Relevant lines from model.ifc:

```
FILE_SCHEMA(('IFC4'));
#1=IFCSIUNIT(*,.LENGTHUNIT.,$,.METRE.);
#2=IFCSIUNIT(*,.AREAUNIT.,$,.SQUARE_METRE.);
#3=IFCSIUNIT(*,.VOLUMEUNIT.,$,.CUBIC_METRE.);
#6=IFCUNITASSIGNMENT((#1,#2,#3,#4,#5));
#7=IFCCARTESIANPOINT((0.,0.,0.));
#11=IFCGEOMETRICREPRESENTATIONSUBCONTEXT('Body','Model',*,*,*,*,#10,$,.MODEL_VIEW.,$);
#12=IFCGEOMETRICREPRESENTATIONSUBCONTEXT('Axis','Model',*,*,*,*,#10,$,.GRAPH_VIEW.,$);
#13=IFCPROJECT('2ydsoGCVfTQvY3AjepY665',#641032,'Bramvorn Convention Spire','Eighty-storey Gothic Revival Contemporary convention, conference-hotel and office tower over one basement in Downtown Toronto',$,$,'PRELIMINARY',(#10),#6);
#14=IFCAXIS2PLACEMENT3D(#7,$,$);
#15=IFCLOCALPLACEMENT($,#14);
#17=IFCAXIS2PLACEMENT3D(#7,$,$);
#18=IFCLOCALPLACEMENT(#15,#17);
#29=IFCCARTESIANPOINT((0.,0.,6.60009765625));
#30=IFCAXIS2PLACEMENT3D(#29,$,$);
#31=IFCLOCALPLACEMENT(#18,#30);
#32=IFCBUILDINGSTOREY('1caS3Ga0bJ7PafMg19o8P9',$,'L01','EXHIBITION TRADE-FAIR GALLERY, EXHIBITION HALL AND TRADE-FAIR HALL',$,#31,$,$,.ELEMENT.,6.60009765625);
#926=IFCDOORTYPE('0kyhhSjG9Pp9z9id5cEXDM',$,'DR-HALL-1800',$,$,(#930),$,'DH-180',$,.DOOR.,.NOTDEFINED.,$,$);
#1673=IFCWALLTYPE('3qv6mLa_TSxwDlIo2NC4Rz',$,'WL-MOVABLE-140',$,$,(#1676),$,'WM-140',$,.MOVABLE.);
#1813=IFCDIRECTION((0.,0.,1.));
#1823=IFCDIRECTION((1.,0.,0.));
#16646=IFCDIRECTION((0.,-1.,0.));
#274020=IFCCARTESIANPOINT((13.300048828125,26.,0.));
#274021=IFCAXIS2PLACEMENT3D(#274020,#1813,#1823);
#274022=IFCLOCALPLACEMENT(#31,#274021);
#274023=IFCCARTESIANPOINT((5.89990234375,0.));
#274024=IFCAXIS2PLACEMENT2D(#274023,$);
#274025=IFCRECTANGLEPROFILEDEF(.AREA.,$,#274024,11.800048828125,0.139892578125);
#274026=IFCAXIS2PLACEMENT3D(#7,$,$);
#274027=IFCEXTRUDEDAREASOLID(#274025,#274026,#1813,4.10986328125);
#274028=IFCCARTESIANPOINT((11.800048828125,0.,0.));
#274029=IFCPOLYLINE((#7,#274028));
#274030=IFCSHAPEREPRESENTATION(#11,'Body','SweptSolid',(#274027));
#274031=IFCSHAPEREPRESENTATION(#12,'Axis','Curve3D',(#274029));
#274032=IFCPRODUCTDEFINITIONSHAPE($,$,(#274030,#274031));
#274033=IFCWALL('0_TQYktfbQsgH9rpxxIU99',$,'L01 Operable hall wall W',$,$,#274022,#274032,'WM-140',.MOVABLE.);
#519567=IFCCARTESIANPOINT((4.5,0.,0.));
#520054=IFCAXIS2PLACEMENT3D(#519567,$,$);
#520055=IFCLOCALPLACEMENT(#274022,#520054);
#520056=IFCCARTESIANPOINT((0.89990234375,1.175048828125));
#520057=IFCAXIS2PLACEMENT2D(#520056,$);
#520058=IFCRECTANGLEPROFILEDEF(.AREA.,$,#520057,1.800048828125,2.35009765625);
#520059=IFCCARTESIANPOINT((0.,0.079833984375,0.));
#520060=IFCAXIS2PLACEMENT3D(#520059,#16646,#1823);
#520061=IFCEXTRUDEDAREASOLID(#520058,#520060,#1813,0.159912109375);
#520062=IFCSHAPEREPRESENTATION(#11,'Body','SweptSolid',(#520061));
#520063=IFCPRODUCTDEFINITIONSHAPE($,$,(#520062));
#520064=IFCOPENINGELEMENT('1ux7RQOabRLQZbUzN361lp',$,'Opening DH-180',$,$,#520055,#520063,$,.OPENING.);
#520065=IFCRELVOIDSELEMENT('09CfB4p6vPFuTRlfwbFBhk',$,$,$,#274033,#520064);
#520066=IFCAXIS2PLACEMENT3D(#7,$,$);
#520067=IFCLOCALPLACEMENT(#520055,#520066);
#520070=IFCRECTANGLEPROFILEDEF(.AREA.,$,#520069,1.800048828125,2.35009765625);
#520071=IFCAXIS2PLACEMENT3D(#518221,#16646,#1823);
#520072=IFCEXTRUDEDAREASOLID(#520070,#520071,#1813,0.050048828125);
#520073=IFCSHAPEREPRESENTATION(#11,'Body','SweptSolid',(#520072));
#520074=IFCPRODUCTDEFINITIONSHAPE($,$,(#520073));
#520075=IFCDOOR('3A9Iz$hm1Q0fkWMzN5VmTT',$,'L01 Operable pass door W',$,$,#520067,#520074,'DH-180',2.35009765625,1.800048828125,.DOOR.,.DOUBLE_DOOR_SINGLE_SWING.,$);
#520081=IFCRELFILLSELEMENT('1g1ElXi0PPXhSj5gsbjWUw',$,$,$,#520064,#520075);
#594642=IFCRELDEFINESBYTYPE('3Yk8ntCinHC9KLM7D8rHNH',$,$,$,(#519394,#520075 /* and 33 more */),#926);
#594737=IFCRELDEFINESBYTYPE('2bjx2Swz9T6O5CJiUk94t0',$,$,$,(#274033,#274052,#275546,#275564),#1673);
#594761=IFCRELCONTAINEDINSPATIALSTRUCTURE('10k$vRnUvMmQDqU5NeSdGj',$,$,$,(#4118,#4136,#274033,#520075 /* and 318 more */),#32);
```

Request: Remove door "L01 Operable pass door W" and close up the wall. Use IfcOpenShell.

```python
import ifcopenshell
import ifcopenshell.api.feature
import ifcopenshell.api.root
import ifcopenshell.geom
import ifcopenshell.util.shape

model = ifcopenshell.open("model.ifc")
settings = ifcopenshell.geom.settings()


def volume(element):
    """Net volume in cubic metres, openings subtracted."""
    shape = ifcopenshell.geom.create_shape(settings, element)
    return ifcopenshell.util.shape.get_volume(shape.geometry)


door = model.by_guid("3A9Iz$hm1Q0fkWMzN5VmTT")
opening = door.FillsVoids[0].RelatingOpeningElement
wall = opening.VoidsElements[0].RelatingBuildingElement
before = volume(wall)

ifcopenshell.api.root.remove_product(model, product=door)
ifcopenshell.api.feature.remove_feature(model, feature=opening)

after = volume(wall)

print(f"wall volume {before:.3f} -> {after:.3f} m3")

model.write("model_v2.ifc")
```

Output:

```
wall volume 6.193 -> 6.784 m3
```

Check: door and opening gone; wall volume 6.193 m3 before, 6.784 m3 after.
